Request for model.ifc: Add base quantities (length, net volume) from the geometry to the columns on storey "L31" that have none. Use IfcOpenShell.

First a look at what the model holds.

```python
import ifcopenshell
import ifcopenshell.util.element
import ifcopenshell.util.unit

model = ifcopenshell.open("model.ifc")
print(model.schema)
for unit_type in ("LENGTHUNIT", "AREAUNIT", "VOLUMEUNIT"):
    print(unit_type, ifcopenshell.util.unit.calculate_unit_scale(model, unit_type))
storey = next(s for s in model.by_type("IfcBuildingStorey") if s.Name == "L31")
columns = [e for e in ifcopenshell.util.element.get_decomposition(storey) if e.is_a("IfcColumn")]
for e in sorted(columns, key=lambda e: e.id()):
    print(e.id(), e.is_a(), e.Name, list(ifcopenshell.util.element.get_psets(e, qtos_only=True)), sep=" | ")
```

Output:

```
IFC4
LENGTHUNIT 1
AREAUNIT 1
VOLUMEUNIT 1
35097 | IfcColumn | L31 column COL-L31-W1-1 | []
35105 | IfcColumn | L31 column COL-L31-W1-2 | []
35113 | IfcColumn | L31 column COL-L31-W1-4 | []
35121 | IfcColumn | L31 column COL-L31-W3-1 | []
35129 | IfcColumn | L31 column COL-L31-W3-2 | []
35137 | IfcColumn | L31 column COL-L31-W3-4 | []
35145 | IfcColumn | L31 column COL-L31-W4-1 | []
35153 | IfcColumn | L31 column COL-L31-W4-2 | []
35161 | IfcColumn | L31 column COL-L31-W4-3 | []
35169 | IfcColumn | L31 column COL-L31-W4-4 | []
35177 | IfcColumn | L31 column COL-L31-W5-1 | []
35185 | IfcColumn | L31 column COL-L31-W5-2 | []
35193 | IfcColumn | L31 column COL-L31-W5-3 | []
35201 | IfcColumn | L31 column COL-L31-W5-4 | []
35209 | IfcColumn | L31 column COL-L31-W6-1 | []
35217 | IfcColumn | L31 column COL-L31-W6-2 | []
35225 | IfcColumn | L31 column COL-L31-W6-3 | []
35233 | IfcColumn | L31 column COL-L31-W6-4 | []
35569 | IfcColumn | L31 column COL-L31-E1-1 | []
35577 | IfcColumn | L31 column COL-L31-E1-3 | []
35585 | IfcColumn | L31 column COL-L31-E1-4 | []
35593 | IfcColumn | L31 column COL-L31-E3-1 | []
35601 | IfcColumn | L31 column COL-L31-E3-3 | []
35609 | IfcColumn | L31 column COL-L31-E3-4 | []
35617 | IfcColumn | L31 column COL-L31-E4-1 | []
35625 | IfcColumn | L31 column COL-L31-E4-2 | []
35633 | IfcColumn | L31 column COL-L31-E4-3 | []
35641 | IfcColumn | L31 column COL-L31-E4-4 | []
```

```python
import ifcopenshell
import ifcopenshell.api.pset
import ifcopenshell.geom
import ifcopenshell.util.element
import ifcopenshell.util.shape
import ifcopenshell.util.unit

model = ifcopenshell.open("model.ifc")
unit_scale = ifcopenshell.util.unit.calculate_unit_scale(model)
volume_scale = ifcopenshell.util.unit.calculate_unit_scale(model, "VOLUMEUNIT")
settings = ifcopenshell.geom.settings()

storey = next(s for s in model.by_type("IfcBuildingStorey") if s.Name == "L31")
columns = [e for e in ifcopenshell.util.element.get_decomposition(storey) if e.is_a("IfcColumn")]

for e in sorted(columns, key=lambda e: e.id()):
    if ifcopenshell.util.element.get_psets(e, qtos_only=True, should_inherit=False):
        continue
    # Geometry comes back in metres, in the element's own axes.
    shape = ifcopenshell.geom.create_shape(settings, e)
    values = {
        "Length": ifcopenshell.util.shape.get_z(shape.geometry) / unit_scale,
        "NetVolume": ifcopenshell.util.shape.get_volume(shape.geometry) / volume_scale,
    }
    qto = ifcopenshell.api.pset.add_qto(model, product=e, name="Qto_ColumnBaseQuantities")
    ifcopenshell.api.pset.edit_qto(model, qto=qto, properties=values)
    print(e.id(), {k: round(v, 3) for k, v in values.items()})

model.write("model_v2.ifc")
```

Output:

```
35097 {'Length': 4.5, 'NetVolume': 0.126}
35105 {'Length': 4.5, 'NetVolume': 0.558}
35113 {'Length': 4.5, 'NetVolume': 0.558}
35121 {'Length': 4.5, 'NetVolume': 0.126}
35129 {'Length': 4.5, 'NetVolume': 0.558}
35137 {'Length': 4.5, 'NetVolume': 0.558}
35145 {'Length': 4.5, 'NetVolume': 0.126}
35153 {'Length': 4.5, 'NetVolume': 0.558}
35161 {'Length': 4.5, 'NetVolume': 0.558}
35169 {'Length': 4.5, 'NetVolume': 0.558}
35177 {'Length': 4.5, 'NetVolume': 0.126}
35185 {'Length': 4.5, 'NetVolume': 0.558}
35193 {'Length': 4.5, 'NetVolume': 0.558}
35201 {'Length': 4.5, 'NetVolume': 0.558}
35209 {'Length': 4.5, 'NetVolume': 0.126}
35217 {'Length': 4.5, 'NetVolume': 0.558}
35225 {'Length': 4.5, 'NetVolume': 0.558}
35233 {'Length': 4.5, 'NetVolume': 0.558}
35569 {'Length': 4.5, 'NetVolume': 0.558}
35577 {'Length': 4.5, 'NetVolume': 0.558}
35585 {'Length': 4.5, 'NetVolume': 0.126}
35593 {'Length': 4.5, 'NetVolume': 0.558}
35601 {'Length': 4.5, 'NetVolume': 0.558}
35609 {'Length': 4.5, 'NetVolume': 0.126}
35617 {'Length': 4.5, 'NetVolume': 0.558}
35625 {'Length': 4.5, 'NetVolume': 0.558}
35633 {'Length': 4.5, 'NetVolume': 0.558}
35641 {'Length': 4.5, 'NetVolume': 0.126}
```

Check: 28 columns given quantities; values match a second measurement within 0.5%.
